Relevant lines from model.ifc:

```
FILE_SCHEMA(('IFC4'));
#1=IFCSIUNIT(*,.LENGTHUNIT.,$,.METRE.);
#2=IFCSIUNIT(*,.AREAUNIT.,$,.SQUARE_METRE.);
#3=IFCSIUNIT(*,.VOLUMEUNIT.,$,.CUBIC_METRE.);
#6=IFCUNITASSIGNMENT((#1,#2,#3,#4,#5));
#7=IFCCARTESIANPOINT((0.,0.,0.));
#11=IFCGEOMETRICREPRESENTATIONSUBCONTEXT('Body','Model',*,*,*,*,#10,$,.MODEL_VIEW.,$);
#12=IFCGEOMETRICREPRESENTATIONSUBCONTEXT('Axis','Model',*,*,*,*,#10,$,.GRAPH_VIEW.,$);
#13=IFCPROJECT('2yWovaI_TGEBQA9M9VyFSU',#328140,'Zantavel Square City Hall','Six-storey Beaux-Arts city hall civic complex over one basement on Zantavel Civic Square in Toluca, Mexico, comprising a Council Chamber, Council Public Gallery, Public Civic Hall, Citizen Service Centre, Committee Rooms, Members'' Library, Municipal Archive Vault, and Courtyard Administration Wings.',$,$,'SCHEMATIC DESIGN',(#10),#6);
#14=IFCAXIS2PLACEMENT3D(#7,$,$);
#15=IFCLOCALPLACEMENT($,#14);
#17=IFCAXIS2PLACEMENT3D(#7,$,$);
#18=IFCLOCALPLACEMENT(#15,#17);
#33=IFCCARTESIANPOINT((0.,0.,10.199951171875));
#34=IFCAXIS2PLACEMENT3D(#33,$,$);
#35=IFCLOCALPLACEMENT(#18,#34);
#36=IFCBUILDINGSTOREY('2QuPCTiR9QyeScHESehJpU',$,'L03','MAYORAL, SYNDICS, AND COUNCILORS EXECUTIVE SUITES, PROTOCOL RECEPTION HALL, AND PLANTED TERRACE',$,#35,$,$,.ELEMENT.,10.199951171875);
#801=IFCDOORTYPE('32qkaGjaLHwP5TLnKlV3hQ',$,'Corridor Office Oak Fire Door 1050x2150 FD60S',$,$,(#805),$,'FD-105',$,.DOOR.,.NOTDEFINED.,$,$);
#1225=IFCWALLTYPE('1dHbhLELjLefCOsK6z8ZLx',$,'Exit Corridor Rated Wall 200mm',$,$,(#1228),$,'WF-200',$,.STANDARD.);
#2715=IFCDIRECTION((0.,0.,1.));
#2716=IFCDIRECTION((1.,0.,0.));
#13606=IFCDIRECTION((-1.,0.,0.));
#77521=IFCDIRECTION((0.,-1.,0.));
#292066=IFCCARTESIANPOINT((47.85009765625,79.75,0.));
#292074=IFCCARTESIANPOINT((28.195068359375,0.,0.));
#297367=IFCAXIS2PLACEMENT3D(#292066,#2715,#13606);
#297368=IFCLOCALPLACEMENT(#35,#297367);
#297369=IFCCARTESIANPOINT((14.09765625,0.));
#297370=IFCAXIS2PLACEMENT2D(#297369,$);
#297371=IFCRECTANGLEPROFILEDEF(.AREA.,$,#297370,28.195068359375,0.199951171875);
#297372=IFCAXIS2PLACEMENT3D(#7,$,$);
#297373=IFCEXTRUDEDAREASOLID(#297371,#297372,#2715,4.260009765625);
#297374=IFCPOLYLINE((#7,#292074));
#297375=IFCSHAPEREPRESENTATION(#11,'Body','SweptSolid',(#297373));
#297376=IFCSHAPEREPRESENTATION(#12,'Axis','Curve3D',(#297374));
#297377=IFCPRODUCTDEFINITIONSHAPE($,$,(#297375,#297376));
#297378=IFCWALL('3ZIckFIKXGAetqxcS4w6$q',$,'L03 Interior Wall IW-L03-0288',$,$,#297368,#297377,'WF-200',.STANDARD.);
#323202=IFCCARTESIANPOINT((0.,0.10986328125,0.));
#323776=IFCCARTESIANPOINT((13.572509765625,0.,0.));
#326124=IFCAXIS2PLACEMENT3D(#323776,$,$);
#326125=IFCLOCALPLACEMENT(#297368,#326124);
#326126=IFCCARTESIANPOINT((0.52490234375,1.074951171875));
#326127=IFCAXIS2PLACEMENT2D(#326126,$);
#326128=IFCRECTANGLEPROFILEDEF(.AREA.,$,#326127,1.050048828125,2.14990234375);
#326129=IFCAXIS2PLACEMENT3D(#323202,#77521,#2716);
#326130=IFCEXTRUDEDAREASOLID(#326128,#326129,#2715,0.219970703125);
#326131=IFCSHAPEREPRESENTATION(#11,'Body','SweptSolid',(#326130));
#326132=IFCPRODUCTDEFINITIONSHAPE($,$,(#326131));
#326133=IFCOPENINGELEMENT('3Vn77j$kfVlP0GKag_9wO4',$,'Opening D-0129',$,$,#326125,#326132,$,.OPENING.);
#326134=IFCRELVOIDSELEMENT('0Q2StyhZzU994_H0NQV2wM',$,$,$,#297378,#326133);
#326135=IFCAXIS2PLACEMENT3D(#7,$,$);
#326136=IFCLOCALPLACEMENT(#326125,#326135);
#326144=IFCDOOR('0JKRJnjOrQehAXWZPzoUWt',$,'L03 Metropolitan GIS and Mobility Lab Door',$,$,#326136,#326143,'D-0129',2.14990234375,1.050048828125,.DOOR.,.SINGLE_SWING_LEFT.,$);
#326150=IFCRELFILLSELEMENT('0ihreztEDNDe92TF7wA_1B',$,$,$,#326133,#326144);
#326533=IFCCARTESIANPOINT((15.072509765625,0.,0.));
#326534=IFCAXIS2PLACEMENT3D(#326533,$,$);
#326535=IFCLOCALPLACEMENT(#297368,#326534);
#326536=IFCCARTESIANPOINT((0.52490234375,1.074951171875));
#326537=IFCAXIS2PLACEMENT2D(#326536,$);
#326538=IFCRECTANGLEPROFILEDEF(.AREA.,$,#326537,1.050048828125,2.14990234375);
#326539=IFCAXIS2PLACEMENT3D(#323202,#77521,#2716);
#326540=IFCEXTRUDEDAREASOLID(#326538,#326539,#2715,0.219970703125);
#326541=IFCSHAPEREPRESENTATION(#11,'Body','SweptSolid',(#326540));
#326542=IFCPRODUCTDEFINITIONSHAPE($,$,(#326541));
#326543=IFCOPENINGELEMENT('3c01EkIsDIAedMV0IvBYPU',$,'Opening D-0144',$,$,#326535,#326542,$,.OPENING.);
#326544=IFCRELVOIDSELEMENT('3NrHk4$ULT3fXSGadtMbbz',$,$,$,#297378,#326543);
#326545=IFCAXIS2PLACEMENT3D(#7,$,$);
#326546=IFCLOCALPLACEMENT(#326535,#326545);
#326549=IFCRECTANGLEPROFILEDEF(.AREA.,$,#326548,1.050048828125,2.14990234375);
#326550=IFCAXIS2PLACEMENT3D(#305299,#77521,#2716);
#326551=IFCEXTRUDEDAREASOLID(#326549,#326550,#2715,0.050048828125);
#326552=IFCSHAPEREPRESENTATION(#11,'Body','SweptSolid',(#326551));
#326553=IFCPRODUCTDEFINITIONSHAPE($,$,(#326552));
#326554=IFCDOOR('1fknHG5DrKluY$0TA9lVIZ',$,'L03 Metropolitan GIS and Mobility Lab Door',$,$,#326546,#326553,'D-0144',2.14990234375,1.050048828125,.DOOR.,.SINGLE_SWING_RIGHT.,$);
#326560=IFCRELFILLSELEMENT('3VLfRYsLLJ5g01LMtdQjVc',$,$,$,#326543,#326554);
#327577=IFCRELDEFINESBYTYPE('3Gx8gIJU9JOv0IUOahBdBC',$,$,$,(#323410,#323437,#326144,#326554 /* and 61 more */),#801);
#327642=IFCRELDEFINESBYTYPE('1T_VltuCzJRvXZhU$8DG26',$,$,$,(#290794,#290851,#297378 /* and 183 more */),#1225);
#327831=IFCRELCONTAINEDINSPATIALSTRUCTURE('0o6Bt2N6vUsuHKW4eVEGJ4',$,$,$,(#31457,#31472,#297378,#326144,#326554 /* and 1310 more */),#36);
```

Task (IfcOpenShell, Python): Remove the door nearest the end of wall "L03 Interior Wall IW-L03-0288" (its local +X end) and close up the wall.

```python
import ifcopenshell
import ifcopenshell.api.feature
import ifcopenshell.api.root
import ifcopenshell.geom
import ifcopenshell.util.shape

model = ifcopenshell.open("model.ifc")
settings = ifcopenshell.geom.settings()


def volume(element):
    """Net volume in cubic metres, openings subtracted."""
    shape = ifcopenshell.geom.create_shape(settings, element)
    return ifcopenshell.util.shape.get_volume(shape.geometry)


door = model.by_guid("1fknHG5DrKluY$0TA9lVIZ")
opening = door.FillsVoids[0].RelatingOpeningElement
wall = opening.VoidsElements[0].RelatingBuildingElement
before = volume(wall)

ifcopenshell.api.root.remove_product(model, product=door)
ifcopenshell.api.feature.remove_feature(model, feature=opening)

after = volume(wall)

print(f"wall volume {before:.3f} -> {after:.3f} m3")

model.write("model_v2.ifc")
```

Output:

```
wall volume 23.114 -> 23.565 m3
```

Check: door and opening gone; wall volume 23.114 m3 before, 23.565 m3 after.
